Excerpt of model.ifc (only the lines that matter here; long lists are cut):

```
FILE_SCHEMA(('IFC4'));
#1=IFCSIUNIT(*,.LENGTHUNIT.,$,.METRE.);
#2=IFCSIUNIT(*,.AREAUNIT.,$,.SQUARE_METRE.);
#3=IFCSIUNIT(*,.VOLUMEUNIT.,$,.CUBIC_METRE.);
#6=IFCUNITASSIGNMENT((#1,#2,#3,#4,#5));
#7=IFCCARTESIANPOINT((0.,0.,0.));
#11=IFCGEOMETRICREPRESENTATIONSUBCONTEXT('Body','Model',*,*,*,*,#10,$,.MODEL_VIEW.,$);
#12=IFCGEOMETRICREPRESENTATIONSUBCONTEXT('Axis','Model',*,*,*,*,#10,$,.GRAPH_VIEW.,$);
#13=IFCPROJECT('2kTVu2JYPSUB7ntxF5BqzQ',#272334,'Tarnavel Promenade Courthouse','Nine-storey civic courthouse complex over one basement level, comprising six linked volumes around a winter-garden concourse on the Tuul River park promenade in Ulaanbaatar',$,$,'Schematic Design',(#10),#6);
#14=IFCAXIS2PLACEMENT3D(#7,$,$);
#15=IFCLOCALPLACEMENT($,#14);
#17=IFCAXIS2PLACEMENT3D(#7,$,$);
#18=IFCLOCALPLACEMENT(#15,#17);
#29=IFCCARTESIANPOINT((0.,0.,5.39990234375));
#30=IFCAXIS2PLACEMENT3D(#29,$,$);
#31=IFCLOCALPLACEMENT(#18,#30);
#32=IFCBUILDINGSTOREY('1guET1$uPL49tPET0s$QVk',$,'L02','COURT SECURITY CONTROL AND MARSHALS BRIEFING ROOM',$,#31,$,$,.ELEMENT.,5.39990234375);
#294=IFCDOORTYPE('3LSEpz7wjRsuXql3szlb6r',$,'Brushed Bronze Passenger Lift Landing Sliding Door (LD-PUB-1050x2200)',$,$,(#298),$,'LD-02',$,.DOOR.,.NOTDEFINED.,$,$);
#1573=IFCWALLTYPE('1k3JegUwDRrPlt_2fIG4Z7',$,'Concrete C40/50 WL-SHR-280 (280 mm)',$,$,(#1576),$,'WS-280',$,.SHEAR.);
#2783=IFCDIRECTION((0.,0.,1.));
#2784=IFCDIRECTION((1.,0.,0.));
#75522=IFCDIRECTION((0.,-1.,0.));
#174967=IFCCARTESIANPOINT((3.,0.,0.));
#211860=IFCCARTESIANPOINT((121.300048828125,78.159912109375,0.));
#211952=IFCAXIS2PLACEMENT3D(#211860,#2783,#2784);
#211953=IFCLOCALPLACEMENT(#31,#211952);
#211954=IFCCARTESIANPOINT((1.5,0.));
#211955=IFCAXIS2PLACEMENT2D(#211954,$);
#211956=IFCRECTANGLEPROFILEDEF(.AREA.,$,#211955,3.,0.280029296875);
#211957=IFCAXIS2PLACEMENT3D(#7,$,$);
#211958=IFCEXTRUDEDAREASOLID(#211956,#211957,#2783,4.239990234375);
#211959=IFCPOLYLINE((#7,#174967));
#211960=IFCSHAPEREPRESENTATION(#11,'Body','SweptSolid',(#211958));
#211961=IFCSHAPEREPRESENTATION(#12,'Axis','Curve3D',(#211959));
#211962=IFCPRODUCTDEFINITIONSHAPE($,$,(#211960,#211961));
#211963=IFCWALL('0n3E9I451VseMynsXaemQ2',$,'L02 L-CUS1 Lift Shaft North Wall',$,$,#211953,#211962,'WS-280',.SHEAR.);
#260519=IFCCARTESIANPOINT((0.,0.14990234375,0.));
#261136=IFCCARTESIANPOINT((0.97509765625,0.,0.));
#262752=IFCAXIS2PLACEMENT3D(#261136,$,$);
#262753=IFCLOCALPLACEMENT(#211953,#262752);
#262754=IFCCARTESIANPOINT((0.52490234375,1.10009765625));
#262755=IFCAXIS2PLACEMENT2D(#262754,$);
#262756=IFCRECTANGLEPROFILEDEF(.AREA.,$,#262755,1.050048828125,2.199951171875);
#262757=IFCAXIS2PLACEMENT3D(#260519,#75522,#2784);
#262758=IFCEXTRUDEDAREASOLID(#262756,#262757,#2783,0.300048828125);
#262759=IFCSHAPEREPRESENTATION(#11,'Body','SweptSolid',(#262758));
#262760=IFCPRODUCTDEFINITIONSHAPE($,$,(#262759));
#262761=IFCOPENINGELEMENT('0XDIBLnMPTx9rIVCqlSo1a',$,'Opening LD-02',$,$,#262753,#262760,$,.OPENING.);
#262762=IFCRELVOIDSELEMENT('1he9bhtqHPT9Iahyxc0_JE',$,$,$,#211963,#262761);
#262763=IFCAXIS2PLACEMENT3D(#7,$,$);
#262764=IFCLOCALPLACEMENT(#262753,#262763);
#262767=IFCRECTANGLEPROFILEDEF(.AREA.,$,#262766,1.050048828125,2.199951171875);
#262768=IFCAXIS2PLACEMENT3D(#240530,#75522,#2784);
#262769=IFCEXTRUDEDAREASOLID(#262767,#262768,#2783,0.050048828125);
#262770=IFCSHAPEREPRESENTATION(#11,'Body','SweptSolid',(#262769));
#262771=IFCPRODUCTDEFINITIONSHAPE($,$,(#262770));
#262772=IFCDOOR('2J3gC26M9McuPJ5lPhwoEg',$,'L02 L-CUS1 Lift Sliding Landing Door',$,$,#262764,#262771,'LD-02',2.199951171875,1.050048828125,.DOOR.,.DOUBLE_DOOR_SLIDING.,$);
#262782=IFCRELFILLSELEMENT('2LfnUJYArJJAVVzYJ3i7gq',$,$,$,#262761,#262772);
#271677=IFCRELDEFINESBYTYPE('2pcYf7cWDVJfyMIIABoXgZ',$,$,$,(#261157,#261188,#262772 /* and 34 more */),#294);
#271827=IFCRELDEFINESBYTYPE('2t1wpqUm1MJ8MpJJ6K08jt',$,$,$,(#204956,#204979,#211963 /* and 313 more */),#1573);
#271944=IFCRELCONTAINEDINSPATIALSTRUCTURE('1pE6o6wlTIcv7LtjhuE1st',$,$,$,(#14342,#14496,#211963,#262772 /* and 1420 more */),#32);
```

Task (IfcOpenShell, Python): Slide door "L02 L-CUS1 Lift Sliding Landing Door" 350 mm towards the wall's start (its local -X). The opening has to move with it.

```python
import ifcopenshell
import ifcopenshell.api.geometry
import ifcopenshell.util.placement
import ifcopenshell.util.unit

model = ifcopenshell.open("model.ifc")
unit_scale = ifcopenshell.util.unit.calculate_unit_scale(model)

door = model.by_guid("2J3gC26M9McuPJ5lPhwoEg")
opening = door.FillsVoids[0].RelatingOpeningElement
wall = opening.VoidsElements[0].RelatingBuildingElement

wall_matrix = ifcopenshell.util.placement.get_local_placement(wall.ObjectPlacement)
shift = wall_matrix[:3, 0] * -0.35 / unit_scale
before = ifcopenshell.util.placement.get_local_placement(door.ObjectPlacement)[:3, 3].copy()

# The door is placed relative to its opening, so it follows when the opening moves.
matrix = ifcopenshell.util.placement.get_local_placement(opening.ObjectPlacement)
matrix[:3, 3] += shift
ifcopenshell.api.geometry.edit_object_placement(
    model, product=opening, matrix=matrix, is_si=False, should_transform_children=True
)

after = ifcopenshell.util.placement.get_local_placement(door.ObjectPlacement)[:3, 3]
print("door moved by", (after - before).round(3) + 0.0)

model.write("model_rev.ifc")
```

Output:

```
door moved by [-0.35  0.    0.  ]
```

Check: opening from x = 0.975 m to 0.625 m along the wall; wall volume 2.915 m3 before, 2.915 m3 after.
